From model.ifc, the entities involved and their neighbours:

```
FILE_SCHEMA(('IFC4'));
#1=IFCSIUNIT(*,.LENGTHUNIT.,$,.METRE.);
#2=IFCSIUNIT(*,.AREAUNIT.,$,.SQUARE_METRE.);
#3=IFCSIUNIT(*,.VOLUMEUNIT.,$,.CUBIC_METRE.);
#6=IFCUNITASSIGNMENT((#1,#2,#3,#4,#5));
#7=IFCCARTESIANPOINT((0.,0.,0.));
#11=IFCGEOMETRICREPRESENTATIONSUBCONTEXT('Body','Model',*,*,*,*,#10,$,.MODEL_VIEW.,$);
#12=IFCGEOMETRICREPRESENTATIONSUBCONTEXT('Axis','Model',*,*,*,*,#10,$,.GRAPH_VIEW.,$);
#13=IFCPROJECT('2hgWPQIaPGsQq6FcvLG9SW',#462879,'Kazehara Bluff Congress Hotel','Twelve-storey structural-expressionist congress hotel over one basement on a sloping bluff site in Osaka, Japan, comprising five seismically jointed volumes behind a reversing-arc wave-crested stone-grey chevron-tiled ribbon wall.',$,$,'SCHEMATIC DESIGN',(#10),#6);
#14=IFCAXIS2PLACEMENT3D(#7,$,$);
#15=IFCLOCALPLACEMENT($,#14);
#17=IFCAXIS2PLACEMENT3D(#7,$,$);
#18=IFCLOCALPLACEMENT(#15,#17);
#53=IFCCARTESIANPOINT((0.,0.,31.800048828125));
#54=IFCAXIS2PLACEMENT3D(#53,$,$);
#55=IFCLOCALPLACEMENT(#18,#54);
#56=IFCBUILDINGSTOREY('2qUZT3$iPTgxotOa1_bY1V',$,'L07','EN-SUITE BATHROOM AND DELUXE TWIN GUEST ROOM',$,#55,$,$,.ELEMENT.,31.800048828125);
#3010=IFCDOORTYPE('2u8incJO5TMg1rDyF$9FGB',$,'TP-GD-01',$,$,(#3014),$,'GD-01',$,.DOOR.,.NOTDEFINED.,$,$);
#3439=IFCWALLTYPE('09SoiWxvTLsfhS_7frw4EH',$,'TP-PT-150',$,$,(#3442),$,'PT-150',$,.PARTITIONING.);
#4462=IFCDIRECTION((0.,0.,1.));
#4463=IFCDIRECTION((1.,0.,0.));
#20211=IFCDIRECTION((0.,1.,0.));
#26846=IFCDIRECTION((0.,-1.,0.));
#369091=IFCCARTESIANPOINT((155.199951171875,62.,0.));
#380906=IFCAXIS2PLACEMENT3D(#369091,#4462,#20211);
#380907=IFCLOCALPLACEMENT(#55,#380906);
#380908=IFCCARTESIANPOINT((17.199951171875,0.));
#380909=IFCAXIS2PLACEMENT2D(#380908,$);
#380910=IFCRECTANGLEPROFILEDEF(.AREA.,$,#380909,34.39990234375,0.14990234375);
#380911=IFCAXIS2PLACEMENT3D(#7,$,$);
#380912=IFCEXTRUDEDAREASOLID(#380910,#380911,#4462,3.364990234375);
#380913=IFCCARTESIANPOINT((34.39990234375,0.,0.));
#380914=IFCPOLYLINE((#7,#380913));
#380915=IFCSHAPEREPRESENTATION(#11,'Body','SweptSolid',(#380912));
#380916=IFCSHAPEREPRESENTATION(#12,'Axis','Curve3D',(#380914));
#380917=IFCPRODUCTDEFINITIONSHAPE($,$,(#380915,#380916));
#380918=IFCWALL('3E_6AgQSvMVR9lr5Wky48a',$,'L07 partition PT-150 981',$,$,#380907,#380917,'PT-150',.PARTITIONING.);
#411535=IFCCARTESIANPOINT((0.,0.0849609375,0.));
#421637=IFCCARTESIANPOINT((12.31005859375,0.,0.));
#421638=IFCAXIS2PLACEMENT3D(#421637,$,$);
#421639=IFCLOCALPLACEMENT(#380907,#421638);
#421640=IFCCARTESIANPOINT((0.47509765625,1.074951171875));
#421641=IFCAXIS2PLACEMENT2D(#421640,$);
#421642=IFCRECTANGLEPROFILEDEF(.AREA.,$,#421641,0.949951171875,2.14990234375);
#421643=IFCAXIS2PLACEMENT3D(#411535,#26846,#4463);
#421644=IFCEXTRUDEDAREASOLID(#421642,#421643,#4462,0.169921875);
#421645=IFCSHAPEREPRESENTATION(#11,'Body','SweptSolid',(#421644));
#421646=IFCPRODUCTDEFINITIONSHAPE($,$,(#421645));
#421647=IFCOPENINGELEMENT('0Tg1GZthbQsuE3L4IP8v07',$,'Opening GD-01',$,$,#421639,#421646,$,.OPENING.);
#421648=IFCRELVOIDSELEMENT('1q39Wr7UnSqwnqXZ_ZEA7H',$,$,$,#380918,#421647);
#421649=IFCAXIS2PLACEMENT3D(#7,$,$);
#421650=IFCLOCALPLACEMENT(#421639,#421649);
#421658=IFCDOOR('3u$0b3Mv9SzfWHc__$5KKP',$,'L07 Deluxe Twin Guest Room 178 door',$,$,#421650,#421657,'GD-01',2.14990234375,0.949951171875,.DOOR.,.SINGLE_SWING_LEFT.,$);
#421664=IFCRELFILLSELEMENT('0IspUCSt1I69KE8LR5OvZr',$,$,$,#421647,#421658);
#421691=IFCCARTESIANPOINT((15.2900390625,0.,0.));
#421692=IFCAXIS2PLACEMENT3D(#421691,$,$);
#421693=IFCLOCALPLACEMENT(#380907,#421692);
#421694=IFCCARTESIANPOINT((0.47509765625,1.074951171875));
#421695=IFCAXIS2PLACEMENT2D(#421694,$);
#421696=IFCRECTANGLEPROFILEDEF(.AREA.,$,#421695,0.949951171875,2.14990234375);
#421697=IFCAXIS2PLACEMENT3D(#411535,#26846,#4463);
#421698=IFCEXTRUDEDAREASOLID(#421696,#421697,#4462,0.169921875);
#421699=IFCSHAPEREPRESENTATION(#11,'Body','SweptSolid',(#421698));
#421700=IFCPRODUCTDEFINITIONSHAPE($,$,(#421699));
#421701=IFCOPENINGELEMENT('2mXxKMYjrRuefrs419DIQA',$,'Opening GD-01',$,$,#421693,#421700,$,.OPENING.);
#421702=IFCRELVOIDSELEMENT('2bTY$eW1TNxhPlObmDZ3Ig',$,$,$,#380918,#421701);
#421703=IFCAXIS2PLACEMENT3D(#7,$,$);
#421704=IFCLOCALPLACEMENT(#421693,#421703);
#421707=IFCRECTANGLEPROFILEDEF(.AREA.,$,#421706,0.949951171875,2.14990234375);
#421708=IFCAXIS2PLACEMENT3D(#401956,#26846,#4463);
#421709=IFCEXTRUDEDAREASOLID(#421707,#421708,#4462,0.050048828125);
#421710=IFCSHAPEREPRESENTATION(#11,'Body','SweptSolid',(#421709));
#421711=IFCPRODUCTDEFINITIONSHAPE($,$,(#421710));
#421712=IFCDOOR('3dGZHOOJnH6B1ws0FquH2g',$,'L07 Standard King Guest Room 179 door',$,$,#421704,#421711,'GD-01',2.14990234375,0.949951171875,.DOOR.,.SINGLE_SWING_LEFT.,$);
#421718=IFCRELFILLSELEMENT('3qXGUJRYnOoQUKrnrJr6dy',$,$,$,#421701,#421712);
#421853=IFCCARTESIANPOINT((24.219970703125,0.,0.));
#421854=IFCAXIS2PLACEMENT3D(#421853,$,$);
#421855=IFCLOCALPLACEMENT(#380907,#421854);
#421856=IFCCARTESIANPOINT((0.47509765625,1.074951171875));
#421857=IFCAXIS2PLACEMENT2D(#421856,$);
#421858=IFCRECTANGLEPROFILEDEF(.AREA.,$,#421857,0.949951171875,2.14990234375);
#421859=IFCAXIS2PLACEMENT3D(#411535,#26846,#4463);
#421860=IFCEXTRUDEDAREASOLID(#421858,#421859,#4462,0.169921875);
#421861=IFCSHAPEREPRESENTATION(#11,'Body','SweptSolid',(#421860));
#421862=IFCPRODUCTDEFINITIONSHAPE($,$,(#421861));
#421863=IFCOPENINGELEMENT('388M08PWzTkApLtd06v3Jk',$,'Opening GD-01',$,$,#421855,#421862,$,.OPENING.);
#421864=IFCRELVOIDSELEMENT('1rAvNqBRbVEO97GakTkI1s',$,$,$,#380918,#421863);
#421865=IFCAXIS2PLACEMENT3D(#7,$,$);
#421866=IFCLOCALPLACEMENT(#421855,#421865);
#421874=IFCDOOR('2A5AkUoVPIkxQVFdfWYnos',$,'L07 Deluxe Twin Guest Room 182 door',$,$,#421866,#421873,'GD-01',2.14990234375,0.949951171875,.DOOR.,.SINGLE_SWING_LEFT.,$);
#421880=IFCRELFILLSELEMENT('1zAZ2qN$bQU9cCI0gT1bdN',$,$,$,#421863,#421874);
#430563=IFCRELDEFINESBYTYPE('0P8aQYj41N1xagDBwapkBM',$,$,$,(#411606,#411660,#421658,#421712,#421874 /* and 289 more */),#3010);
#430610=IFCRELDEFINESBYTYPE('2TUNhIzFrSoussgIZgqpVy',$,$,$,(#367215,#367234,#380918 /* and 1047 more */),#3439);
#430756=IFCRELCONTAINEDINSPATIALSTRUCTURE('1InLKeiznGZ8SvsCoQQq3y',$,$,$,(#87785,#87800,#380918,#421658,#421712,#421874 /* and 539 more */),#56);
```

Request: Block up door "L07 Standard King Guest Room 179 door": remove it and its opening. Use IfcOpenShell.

```python
import ifcopenshell
import ifcopenshell.api.feature
import ifcopenshell.api.root
import ifcopenshell.geom
import ifcopenshell.util.shape

model = ifcopenshell.open("model.ifc")
settings = ifcopenshell.geom.settings()


def volume(element):
    """Net volume in cubic metres, openings subtracted."""
    shape = ifcopenshell.geom.create_shape(settings, element)
    return ifcopenshell.util.shape.get_volume(shape.geometry)


door = model.by_guid("3dGZHOOJnH6B1ws0FquH2g")
opening = door.FillsVoids[0].RelatingOpeningElement
wall = opening.VoidsElements[0].RelatingBuildingElement
before = volume(wall)

ifcopenshell.api.root.remove_product(model, product=door)
ifcopenshell.api.feature.remove_feature(model, feature=opening)

after = volume(wall)

print(f"wall volume {before:.3f} -> {after:.3f} m3")

model.write("model_v2.ifc")
```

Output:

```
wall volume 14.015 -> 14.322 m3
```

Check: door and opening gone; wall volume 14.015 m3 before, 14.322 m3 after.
